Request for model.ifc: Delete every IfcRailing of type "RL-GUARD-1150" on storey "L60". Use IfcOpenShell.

First a look at what the model holds.

```python
import ifcopenshell
import ifcopenshell.util.element

model = ifcopenshell.open("model.ifc")
print(model.schema)
storey = next(s for s in model.by_type("IfcBuildingStorey") if s.Name == "L60")
railings = [e for e in ifcopenshell.util.element.get_decomposition(storey) if e.is_a("IfcRailing")]
seen = {}
for e in railings:
    element_type = ifcopenshell.util.element.get_type(e)
    name = element_type.Name if element_type not in (None, e) else None
    seen[name] = seen.get(name, 0) + 1
for name, count in sorted(seen.items(), key=str):
    print(count, "x", name)
```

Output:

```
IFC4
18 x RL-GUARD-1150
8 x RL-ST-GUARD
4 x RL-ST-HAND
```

```python
import ifcopenshell
import ifcopenshell.api.root
import ifcopenshell.util.element

model = ifcopenshell.open("model.ifc")

storey = next(s for s in model.by_type("IfcBuildingStorey") if s.Name == "L60")
railings = [e for e in ifcopenshell.util.element.get_decomposition(storey) if e.is_a("IfcRailing")]
targets = [e for e in railings if (t := ifcopenshell.util.element.get_type(e)) not in (None, e) and t.Name == "RL-GUARD-1150"]

for e in targets:
    ifcopenshell.api.root.remove_product(model, product=e)
print(len(targets), "removed")

model.write("model_v2.ifc")
```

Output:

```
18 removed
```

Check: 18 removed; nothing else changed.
